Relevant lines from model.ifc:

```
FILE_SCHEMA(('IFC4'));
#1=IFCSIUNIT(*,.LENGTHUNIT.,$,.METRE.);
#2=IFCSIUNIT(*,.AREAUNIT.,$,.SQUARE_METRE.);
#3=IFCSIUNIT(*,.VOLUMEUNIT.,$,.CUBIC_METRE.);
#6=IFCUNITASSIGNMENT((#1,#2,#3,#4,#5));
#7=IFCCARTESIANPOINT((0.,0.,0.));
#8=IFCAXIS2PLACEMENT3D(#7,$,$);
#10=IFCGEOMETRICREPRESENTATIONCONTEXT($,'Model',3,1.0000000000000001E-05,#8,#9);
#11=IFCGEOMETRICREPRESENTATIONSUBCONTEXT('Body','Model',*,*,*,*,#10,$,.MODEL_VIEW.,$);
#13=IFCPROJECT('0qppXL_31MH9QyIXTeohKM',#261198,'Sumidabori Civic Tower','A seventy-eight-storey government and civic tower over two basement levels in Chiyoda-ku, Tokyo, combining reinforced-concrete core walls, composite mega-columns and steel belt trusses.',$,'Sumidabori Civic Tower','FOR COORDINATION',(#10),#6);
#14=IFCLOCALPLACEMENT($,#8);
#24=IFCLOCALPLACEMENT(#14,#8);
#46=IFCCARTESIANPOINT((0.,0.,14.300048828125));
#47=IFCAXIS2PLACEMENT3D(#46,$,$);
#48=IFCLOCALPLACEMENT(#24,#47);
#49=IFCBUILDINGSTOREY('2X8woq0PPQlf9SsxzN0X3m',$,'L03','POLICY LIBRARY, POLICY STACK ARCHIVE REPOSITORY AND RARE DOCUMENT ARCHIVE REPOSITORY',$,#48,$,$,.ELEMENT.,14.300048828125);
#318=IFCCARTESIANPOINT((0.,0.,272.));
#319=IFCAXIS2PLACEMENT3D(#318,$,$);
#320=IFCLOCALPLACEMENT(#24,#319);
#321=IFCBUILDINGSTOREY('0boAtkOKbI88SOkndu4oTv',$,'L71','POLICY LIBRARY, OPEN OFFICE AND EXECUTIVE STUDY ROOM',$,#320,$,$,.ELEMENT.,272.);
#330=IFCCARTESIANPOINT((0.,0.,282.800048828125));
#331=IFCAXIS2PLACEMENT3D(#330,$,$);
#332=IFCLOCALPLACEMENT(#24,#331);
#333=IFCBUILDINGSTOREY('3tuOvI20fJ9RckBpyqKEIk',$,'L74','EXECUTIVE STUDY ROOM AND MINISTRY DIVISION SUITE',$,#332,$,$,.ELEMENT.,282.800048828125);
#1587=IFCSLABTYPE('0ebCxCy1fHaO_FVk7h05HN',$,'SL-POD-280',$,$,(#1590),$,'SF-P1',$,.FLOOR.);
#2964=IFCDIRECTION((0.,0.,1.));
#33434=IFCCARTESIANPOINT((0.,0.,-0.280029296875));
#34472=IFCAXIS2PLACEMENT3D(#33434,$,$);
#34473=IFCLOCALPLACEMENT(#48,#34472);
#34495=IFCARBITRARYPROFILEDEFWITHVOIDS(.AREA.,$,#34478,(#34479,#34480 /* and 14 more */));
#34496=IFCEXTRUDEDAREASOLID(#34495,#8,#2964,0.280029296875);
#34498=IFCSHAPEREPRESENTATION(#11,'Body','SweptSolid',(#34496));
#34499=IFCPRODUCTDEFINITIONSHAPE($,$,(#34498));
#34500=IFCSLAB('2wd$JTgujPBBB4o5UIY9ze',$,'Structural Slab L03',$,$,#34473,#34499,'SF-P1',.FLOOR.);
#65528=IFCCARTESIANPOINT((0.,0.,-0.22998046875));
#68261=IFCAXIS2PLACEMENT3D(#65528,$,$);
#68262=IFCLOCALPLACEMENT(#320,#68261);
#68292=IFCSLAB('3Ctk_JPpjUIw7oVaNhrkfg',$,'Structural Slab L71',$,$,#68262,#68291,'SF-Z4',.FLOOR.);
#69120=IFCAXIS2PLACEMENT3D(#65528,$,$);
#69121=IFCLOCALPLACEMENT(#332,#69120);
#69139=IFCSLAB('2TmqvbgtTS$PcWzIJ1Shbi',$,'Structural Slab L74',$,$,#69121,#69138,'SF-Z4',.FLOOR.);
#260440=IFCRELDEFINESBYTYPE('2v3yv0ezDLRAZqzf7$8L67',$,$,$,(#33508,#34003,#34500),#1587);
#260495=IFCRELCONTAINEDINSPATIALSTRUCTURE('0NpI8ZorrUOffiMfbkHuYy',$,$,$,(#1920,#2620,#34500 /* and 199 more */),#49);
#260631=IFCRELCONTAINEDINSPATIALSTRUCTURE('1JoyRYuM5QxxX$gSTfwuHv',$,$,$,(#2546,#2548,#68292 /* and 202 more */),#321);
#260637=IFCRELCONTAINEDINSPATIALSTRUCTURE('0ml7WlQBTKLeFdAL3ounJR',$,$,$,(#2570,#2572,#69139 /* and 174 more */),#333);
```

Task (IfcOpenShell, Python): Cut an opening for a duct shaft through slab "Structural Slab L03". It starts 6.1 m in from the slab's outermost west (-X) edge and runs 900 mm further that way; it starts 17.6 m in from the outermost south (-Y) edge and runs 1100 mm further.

```python
import numpy as np
import ifcopenshell
import ifcopenshell.api.feature
import ifcopenshell.api.geometry
import ifcopenshell.api.root
import ifcopenshell.geom
import ifcopenshell.util.placement
import ifcopenshell.util.representation
import ifcopenshell.util.shape
import ifcopenshell.util.unit

model = ifcopenshell.open("model.ifc")
unit_scale = ifcopenshell.util.unit.calculate_unit_scale(model)
settings = ifcopenshell.geom.settings()


def volume(element):
    """Net volume in cubic metres, openings subtracted."""
    shape = ifcopenshell.geom.create_shape(settings, element)
    return ifcopenshell.util.shape.get_volume(shape.geometry)


slab = model.by_guid("2wd$JTgujPBBB4o5UIY9ze")
before = volume(slab)

# Extent in the slab's own axes, in metres. The edges named are its -X and -Y sides.
slab_shape = ifcopenshell.geom.create_shape(settings, slab)
vertices = ifcopenshell.util.shape.get_vertices(slab_shape.geometry)
x_min, y_min, bottom = vertices.min(axis=0)
top = vertices[:, 2].max()

opening = ifcopenshell.api.root.create_entity(model, ifc_class="IfcOpeningElement", name="Duct shaft opening", predefined_type="OPENING")
context = ifcopenshell.util.representation.get_context(model, "Model", "Body", "MODEL_VIEW")
width, depth = 0.9, 1.1
outline = [(0.0, 0.0), (width, 0.0), (width, depth), (0.0, depth), (0.0, 0.0)]
# Overshoot both faces by 50 mm so the cut is clean.
shape = ifcopenshell.api.geometry.add_slab_representation(
    model, context=context, depth=top - bottom + 0.1, polyline=outline
)
ifcopenshell.api.geometry.assign_representation(model, product=opening, representation=shape)

matrix = ifcopenshell.util.placement.get_local_placement(slab.ObjectPlacement)
matrix[:, 3] = matrix @ np.append(np.array([x_min + 6.1, y_min + 17.6, bottom - 0.05]) / unit_scale, 1.0)
ifcopenshell.api.geometry.edit_object_placement(model, product=opening, matrix=matrix, is_si=False)
ifcopenshell.api.feature.add_feature(model, feature=opening, element=slab)

after = volume(slab)

print(f"slab volume {before:.3f} -> {after:.3f} m3")

model.write("model_v2.ifc")
```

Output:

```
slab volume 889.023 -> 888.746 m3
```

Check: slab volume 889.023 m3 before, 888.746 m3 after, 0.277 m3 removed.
